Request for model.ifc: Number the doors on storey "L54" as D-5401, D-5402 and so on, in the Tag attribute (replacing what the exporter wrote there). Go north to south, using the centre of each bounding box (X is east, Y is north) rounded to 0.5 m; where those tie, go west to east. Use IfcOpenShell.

First a look at what the model holds.

```python
import ifcopenshell
import ifcopenshell.util.element
import ifcopenshell.util.placement

model = ifcopenshell.open("model.ifc")
print(model.schema)
storey = next(s for s in model.by_type("IfcBuildingStorey") if s.Name == "L54")
doors = [e for e in ifcopenshell.util.element.get_decomposition(storey) if e.is_a("IfcDoor")]
for e in sorted(doors, key=lambda e: e.id()):
    origin = ifcopenshell.util.placement.get_local_placement(e.ObjectPlacement)[:3, 3]
    print(e.id(), e.Tag, e.Name, origin.round(2) + 0.0, sep=" | ")
```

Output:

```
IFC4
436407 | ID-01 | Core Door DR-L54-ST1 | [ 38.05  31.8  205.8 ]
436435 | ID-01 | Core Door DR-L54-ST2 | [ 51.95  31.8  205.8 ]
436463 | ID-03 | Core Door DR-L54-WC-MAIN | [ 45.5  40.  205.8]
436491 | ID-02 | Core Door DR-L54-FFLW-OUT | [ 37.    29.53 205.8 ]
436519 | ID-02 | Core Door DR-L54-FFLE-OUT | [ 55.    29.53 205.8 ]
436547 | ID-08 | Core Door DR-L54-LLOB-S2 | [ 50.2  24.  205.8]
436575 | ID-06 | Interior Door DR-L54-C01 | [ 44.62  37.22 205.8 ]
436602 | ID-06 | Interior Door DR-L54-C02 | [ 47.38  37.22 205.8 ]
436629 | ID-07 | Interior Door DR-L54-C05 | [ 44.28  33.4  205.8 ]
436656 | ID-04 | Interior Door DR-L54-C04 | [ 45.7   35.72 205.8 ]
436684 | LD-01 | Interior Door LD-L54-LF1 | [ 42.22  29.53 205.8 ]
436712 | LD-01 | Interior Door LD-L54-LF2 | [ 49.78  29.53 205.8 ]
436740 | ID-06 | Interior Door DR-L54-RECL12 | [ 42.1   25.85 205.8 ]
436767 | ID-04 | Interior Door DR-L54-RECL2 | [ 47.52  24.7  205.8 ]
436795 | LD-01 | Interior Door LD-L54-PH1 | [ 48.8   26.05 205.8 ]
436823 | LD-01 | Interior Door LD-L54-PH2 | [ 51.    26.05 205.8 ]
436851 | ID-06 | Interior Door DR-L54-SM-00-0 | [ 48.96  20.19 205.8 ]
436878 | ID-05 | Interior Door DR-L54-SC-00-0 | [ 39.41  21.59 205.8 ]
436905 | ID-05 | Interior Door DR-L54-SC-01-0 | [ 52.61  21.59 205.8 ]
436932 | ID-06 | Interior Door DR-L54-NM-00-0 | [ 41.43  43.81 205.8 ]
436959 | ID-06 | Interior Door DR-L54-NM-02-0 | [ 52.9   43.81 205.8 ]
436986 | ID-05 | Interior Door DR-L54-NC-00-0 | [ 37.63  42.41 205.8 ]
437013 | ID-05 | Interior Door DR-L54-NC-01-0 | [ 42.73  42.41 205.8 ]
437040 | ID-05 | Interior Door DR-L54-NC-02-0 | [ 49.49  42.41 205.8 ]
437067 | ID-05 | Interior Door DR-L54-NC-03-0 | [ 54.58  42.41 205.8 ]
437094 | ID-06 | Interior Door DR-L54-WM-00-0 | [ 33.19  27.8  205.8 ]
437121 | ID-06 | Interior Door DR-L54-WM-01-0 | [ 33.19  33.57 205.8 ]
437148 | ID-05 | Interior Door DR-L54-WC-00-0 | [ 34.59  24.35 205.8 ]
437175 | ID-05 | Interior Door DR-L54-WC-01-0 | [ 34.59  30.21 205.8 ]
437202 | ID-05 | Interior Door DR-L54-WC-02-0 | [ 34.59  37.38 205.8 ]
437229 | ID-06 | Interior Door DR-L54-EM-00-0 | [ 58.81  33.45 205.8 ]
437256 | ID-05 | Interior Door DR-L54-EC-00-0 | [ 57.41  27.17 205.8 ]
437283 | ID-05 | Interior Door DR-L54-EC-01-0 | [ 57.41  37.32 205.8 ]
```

```python
import ifcopenshell
import ifcopenshell.geom
import ifcopenshell.util.element
import ifcopenshell.util.shape

model = ifcopenshell.open("model.ifc")
settings = ifcopenshell.geom.settings()
settings.set("use-world-coords", True)


def centre(element):
    shape = ifcopenshell.geom.create_shape(settings, element)
    return ifcopenshell.util.shape.get_bbox_centroid(shape.geometry)


storey = next(s for s in model.by_type("IfcBuildingStorey") if s.Name == "L54")
doors = [e for e in ifcopenshell.util.element.get_decomposition(storey) if e.is_a("IfcDoor")]

# Insertion points can sit at a corner or the storey origin, so sort by the geometry (in metres).
centres = {e: centre(e) for e in doors}
doors.sort(key=lambda e: (-round(centres[e][1] / 0.5), centres[e][0]))

for i, e in enumerate(doors, start=1):
    number = f"D-54{i:02d}"
    e.Tag = number
    print(e.id(), number)

model.write("model-out.ifc")
```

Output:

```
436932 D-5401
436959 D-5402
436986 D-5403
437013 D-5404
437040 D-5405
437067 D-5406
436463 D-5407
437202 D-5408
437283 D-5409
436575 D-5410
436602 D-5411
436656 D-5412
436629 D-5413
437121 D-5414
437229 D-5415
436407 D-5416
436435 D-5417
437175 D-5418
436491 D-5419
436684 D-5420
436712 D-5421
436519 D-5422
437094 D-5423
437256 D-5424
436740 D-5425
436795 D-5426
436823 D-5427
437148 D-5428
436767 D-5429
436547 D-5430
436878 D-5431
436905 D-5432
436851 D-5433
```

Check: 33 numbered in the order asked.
